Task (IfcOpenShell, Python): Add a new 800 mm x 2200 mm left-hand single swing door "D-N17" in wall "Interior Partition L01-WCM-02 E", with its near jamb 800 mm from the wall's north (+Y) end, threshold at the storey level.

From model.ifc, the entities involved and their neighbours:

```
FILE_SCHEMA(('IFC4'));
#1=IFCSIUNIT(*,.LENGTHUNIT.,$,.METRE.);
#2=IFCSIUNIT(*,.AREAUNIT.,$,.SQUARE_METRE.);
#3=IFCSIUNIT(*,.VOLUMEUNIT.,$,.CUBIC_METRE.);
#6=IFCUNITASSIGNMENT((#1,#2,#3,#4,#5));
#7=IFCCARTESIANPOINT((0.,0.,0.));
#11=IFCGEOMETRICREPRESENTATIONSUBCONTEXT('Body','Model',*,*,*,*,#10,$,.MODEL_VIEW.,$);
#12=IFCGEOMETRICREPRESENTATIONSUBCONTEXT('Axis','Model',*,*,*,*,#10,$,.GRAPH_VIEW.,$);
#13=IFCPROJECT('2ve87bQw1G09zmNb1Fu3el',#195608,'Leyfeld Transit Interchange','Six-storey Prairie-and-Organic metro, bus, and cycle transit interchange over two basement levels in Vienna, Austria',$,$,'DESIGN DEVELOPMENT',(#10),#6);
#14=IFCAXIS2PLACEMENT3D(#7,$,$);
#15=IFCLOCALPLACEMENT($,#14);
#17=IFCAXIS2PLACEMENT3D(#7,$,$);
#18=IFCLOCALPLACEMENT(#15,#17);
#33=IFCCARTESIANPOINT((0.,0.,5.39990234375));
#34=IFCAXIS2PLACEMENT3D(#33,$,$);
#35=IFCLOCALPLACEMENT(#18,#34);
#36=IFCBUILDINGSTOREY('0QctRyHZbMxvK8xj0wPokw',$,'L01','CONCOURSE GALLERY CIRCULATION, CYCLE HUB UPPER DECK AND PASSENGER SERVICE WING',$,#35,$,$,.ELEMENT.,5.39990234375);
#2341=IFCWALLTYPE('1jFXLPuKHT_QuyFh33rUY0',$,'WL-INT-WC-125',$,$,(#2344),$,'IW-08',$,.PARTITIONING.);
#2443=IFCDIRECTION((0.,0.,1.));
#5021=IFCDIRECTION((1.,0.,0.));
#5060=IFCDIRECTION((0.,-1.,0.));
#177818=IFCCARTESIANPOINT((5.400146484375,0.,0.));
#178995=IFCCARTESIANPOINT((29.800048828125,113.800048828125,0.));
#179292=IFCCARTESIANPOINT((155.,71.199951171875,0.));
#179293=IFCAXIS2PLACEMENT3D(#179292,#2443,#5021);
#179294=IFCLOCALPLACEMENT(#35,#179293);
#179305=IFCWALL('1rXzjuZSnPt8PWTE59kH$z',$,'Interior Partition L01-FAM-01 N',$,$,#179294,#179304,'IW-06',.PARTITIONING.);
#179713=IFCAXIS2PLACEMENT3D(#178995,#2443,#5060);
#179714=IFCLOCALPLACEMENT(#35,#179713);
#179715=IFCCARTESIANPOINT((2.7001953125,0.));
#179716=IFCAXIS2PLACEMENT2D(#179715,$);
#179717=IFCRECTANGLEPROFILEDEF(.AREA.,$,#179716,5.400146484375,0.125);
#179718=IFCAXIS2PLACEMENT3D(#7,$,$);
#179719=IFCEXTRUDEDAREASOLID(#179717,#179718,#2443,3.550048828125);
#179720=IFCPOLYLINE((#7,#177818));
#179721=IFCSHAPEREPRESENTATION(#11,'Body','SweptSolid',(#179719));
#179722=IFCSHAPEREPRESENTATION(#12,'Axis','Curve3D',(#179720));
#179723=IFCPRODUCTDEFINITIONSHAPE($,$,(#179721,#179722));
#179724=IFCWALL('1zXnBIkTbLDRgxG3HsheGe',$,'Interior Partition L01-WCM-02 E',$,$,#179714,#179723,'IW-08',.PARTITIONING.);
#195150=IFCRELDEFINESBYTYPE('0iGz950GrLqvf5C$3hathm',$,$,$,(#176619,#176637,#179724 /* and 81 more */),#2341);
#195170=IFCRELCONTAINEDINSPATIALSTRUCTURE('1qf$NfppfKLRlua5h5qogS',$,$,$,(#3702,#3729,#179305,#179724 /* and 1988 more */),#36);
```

```python
import numpy as np
import ifcopenshell
import ifcopenshell.api.feature
import ifcopenshell.api.geometry
import ifcopenshell.api.root
import ifcopenshell.api.spatial
import ifcopenshell.geom
import ifcopenshell.util.element
import ifcopenshell.util.placement
import ifcopenshell.util.representation
import ifcopenshell.util.shape
import ifcopenshell.util.unit

model = ifcopenshell.open("model.ifc")
unit_scale = ifcopenshell.util.unit.calculate_unit_scale(model)
settings = ifcopenshell.geom.settings()


def volume(element):
    """Net volume in cubic metres, openings subtracted."""
    shape = ifcopenshell.geom.create_shape(settings, element)
    return ifcopenshell.util.shape.get_volume(shape.geometry)


wall = model.by_guid("1zXnBIkTbLDRgxG3HsheGe")
storey = ifcopenshell.util.element.get_container(wall, ifc_class="IfcBuildingStorey")
context = ifcopenshell.util.representation.get_context(model, "Model", "Body", "MODEL_VIEW")
before = volume(wall)

width, height, from_end, sill = 0.8, 2.2, 0.8, 0.0  # metres

# The wall runs along its own X axis, and the end named is its -X end.
wall_shape = ifcopenshell.geom.create_shape(settings, wall)
x, y, z = ifcopenshell.util.shape.get_vertices(wall_shape.geometry).T
start = x.min() + from_end
face, thickness = float(y.min()), float(y.max() - y.min())
wall_matrix = ifcopenshell.util.placement.get_local_placement(wall.ObjectPlacement)
level = ifcopenshell.util.placement.get_local_placement(storey.ObjectPlacement)[2, 3]


def in_wall(x, y):
    """Placement at x, y metres in the wall's axes, at sill height."""
    matrix = wall_matrix.copy()
    matrix[:, 3] = wall_matrix @ np.array([x / unit_scale, y / unit_scale, 0.0, 1.0])
    matrix[2, 3] = level + sill / unit_scale
    return matrix


# Opening: a box that overshoots both wall faces by 50 mm.
opening = ifcopenshell.api.root.create_entity(model, ifc_class="IfcOpeningElement", predefined_type="OPENING")
box = ifcopenshell.api.geometry.add_wall_representation(
    model, context=context, length=width, height=height, thickness=thickness + 0.1
)
ifcopenshell.api.geometry.assign_representation(model, product=opening, representation=box)
ifcopenshell.api.geometry.edit_object_placement(model, product=opening, matrix=in_wall(start, face - 0.05), is_si=False)
ifcopenshell.api.feature.add_feature(model, feature=opening, element=wall)

door = ifcopenshell.api.root.create_entity(model, ifc_class="IfcDoor", name="D-N17", predefined_type="DOOR")
door.OverallWidth, door.OverallHeight = width / unit_scale, height / unit_scale
door.OperationType = "SINGLE_SWING_LEFT"
body = ifcopenshell.api.geometry.add_door_representation(
    model,
    context=context,
    overall_width=door.OverallWidth,
    overall_height=door.OverallHeight,
    operation_type="SINGLE_SWING_LEFT",
    lining_properties={"LiningDepth": thickness / unit_scale, "ThresholdDepth": thickness / unit_scale},
)
ifcopenshell.api.geometry.assign_representation(model, product=door, representation=body)
ifcopenshell.api.spatial.assign_container(model, products=[door], relating_structure=storey)
ifcopenshell.api.feature.add_filling(model, opening=opening, element=door)

# The lining spans the wall, so the door starts at the wall face.
ifcopenshell.api.geometry.edit_object_placement(model, product=door, matrix=in_wall(start, face), is_si=False)

after = volume(wall)

print(f"wall volume {before:.3f} -> {after:.3f} m3")

model.write("model_edited.ifc")
```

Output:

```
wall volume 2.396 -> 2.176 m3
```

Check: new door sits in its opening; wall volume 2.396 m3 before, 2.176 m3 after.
